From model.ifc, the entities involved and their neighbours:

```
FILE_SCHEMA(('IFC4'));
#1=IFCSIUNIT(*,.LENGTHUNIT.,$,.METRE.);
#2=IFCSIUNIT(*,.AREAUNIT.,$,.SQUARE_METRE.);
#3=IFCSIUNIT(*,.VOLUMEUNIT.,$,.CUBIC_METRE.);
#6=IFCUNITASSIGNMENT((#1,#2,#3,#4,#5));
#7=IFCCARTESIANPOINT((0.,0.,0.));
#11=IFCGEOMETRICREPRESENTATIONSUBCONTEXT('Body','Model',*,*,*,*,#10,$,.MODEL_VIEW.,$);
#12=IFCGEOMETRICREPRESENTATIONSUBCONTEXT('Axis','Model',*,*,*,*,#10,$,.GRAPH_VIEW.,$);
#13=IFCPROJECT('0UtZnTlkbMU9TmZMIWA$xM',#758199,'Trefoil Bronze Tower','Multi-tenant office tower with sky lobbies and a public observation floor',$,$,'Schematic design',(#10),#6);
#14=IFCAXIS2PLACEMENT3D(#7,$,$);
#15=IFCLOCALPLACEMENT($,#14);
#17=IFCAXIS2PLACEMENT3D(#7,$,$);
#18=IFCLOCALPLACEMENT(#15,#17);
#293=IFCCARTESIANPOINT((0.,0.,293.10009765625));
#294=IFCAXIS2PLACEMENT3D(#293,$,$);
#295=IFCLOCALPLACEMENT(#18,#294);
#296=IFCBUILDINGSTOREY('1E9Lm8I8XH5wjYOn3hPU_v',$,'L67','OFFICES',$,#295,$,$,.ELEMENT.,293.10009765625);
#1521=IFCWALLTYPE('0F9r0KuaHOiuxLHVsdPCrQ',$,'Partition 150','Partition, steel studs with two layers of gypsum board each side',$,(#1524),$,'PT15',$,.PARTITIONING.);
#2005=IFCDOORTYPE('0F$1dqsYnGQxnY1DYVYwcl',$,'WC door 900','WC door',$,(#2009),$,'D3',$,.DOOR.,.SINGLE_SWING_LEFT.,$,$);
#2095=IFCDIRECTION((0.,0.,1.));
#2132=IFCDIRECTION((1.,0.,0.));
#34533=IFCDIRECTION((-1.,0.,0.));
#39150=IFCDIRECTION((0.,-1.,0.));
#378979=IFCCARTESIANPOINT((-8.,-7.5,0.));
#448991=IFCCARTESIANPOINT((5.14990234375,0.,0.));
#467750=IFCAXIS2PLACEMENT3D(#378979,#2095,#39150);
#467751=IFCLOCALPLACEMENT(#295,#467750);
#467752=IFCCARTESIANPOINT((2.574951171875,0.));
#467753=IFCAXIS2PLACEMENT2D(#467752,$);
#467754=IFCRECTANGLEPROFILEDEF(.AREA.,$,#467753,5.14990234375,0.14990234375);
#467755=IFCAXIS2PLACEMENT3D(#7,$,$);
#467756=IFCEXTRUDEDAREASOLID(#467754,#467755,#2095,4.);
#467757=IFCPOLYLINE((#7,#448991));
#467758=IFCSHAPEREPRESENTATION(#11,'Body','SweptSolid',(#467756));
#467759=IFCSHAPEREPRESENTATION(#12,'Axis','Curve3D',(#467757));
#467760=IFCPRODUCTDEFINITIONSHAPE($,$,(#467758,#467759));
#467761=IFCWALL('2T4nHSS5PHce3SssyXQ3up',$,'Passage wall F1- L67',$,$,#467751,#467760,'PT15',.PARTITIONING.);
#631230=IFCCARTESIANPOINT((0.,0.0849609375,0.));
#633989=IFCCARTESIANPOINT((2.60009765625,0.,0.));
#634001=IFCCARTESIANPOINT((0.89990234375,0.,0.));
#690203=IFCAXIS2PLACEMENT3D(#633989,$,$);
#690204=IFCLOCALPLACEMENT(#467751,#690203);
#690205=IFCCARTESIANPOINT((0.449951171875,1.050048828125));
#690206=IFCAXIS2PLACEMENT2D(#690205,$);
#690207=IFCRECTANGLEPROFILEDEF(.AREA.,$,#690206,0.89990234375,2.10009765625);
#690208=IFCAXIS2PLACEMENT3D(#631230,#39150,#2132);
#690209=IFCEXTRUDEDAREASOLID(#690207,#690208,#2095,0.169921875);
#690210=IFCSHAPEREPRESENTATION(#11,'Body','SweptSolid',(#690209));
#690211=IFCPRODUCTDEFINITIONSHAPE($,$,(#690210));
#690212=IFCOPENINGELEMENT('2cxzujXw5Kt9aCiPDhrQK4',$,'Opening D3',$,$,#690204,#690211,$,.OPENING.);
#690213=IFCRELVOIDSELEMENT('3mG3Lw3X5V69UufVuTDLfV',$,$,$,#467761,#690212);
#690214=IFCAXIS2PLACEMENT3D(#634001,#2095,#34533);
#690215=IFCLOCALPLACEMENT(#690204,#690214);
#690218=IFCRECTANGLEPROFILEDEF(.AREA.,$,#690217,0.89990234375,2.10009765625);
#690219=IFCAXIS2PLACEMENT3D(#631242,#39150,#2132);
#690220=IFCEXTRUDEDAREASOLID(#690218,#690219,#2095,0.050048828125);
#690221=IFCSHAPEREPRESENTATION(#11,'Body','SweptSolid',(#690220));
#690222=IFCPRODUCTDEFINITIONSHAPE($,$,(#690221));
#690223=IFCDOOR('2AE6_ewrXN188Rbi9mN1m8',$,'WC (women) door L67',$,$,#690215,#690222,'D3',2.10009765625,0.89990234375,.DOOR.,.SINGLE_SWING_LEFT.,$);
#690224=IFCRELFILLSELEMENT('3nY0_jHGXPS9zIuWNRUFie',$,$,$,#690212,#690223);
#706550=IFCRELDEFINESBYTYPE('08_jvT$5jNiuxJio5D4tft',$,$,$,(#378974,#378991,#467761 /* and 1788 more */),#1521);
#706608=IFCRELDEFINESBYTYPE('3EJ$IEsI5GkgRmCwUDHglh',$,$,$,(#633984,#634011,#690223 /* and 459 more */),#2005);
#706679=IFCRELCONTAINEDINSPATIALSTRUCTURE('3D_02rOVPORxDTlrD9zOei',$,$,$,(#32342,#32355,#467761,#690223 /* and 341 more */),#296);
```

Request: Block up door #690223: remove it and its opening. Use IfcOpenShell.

```python
import ifcopenshell
import ifcopenshell.api.feature
import ifcopenshell.api.root
import ifcopenshell.geom
import ifcopenshell.util.shape

model = ifcopenshell.open("model.ifc")
settings = ifcopenshell.geom.settings()


def volume(element):
    """Net volume in cubic metres, openings subtracted."""
    shape = ifcopenshell.geom.create_shape(settings, element)
    return ifcopenshell.util.shape.get_volume(shape.geometry)


door = model.by_guid("2AE6_ewrXN188Rbi9mN1m8")
opening = door.FillsVoids[0].RelatingOpeningElement
wall = opening.VoidsElements[0].RelatingBuildingElement
before = volume(wall)

ifcopenshell.api.root.remove_product(model, product=door)
ifcopenshell.api.feature.remove_feature(model, feature=opening)

after = volume(wall)

print(f"wall volume {before:.3f} -> {after:.3f} m3")

model.write("model_v2.ifc")
```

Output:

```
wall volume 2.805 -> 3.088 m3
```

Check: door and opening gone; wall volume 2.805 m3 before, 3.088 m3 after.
